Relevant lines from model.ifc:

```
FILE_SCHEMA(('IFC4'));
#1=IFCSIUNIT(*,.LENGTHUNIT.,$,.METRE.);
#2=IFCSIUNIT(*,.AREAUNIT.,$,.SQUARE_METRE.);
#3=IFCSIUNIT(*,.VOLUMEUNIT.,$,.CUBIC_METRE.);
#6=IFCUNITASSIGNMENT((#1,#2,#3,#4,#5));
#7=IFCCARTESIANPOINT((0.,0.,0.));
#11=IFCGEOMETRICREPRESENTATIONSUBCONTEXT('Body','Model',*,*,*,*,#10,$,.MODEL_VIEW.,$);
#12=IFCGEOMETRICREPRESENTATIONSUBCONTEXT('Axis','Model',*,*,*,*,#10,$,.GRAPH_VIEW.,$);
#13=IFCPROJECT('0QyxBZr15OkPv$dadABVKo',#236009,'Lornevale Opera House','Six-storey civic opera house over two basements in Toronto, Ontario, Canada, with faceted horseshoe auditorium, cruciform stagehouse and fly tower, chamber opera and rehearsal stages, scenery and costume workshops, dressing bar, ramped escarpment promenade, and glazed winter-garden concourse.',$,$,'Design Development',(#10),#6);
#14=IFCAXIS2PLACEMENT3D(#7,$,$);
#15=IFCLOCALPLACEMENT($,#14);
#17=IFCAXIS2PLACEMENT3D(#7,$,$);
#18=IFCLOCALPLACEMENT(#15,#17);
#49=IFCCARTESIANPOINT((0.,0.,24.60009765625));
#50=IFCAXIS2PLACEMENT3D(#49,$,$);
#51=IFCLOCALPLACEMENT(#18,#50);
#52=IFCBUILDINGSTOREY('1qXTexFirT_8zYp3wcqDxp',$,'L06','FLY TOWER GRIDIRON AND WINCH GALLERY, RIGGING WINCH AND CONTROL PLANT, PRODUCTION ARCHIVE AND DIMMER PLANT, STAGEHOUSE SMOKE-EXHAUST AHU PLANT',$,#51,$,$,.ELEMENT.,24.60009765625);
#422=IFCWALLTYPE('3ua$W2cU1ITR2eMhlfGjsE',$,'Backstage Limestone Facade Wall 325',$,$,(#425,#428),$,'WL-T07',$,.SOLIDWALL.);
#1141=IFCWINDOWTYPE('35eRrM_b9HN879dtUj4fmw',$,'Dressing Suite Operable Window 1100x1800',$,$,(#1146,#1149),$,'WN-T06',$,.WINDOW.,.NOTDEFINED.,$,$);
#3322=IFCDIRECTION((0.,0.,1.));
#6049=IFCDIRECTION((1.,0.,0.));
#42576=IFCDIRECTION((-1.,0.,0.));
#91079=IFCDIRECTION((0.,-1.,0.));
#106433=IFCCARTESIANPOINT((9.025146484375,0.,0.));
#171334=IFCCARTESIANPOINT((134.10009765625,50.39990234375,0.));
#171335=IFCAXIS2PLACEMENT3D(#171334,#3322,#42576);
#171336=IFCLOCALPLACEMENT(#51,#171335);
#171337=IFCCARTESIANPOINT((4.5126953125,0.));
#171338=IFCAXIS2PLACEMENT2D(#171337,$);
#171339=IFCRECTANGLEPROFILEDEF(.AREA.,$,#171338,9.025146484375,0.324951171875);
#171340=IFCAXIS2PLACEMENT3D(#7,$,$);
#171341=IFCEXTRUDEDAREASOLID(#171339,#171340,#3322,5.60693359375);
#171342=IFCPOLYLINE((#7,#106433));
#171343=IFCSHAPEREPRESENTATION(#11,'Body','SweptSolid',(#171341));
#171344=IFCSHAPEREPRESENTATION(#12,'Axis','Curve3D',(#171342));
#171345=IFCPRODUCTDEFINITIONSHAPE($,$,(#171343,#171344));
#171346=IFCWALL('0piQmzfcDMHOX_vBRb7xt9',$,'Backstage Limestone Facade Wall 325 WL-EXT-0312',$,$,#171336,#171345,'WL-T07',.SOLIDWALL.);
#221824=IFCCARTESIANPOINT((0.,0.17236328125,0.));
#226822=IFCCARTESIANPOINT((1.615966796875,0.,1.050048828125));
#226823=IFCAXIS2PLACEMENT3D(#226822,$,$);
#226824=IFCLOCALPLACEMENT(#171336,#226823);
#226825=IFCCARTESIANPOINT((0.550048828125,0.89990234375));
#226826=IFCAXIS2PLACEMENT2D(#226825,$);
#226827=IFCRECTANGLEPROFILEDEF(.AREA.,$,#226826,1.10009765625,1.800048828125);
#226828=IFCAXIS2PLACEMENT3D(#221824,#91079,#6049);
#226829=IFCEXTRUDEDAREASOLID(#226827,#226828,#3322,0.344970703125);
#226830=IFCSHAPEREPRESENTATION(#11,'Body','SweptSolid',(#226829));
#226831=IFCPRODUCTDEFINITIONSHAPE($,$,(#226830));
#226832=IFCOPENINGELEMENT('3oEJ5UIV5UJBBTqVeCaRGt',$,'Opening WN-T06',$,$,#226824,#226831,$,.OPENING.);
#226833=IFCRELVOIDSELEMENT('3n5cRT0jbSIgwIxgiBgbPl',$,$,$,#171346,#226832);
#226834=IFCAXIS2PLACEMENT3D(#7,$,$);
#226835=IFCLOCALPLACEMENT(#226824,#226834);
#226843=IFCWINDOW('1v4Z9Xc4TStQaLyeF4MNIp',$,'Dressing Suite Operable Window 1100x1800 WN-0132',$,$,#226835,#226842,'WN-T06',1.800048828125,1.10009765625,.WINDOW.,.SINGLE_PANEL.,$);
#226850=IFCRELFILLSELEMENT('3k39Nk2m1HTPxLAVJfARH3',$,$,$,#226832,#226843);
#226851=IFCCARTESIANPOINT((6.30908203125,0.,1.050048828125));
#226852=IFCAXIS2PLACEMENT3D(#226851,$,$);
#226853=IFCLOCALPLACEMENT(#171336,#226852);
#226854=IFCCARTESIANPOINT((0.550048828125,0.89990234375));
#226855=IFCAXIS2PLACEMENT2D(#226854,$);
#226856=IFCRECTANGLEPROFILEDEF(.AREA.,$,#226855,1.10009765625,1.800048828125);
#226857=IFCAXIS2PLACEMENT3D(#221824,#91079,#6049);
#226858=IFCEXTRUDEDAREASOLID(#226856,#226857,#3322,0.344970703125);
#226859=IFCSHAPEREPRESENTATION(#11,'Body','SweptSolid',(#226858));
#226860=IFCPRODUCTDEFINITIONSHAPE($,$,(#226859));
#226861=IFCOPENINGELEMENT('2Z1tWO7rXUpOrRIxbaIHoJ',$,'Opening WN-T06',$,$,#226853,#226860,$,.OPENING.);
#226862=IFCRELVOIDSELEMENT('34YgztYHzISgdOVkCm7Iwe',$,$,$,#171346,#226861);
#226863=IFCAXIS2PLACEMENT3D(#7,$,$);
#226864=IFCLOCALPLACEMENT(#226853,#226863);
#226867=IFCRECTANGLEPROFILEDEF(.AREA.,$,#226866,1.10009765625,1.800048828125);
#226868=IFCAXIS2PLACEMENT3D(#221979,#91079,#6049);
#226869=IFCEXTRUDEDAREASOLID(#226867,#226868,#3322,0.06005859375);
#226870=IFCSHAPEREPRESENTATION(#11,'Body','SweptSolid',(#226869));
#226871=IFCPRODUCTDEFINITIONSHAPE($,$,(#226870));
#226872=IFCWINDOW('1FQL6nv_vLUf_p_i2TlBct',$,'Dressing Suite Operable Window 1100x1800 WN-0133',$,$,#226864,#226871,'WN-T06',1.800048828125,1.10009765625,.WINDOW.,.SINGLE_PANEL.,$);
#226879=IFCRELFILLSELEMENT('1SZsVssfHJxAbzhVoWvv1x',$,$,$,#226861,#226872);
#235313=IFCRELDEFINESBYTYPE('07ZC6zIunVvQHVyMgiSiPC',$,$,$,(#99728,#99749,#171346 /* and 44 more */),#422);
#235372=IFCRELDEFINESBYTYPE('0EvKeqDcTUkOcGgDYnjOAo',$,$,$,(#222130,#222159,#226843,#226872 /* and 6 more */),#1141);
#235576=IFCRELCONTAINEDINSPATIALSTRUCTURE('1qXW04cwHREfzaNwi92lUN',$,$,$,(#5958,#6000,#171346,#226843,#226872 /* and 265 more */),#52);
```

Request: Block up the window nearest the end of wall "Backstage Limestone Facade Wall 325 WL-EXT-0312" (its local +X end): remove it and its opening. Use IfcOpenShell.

```python
import ifcopenshell
import ifcopenshell.api.feature
import ifcopenshell.api.root
import ifcopenshell.geom
import ifcopenshell.util.shape

model = ifcopenshell.open("model.ifc")
settings = ifcopenshell.geom.settings()


def volume(element):
    """Net volume in cubic metres, openings subtracted."""
    shape = ifcopenshell.geom.create_shape(settings, element)
    return ifcopenshell.util.shape.get_volume(shape.geometry)


window = model.by_id(226872)
opening = window.FillsVoids[0].RelatingOpeningElement
wall = opening.VoidsElements[0].RelatingBuildingElement
before = volume(wall)

ifcopenshell.api.root.remove_product(model, product=window)
ifcopenshell.api.feature.remove_feature(model, feature=opening)

after = volume(wall)

print(f"wall volume {before:.3f} -> {after:.3f} m3")

model.write("model-out.ifc")
```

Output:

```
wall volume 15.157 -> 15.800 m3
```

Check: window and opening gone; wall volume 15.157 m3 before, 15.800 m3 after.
